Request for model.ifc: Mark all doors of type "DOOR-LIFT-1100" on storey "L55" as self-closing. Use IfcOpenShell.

First a look at what the model holds.

```python
import ifcopenshell
import ifcopenshell.util.element

model = ifcopenshell.open("model.ifc")
print(model.schema)
storey = next(s for s in model.by_type("IfcBuildingStorey") if s.Name == "L55")
doors = [e for e in ifcopenshell.util.element.get_decomposition(storey) if e.is_a("IfcDoor")]
seen = {}
for e in doors:
    element_type = ifcopenshell.util.element.get_type(e)
    key = (element_type.Name if element_type != e and element_type else None, ifcopenshell.util.element.get_pset(e, "Pset_DoorCommon", "SelfClosing"))
    seen[key] = seen.get(key, 0) + 1
for (name, value), count in sorted(seen.items(), key=str):
    print(count, "x", name, "|", value)
```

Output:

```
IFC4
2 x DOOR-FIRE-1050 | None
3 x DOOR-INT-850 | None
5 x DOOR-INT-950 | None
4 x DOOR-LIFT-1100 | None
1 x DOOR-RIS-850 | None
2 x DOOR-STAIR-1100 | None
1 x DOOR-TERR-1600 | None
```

```python
import ifcopenshell
import ifcopenshell.api.pset
import ifcopenshell.util.element

model = ifcopenshell.open("model.ifc")

storey = next(s for s in model.by_type("IfcBuildingStorey") if s.Name == "L55")
doors = [e for e in ifcopenshell.util.element.get_decomposition(storey) if e.is_a("IfcDoor")]

count = 0
for e in doors:
    element_type = ifcopenshell.util.element.get_type(e)
    if element_type in (None, e) or element_type.Name != "DOOR-LIFT-1100":
        continue
    found = ifcopenshell.util.element.get_pset(e, "Pset_DoorCommon", should_inherit=False)
    if found:
        pset = model.by_id(found["id"])
        if len(ifcopenshell.util.element.get_elements_by_pset(pset)) > 1:
            pset = ifcopenshell.api.pset.unshare_pset(model, products=[e], pset=pset)[0]
    else:
        pset = ifcopenshell.api.pset.add_pset(model, product=e, name="Pset_DoorCommon")
    ifcopenshell.api.pset.edit_pset(model, pset=pset, properties={"SelfClosing": True})
    count += 1

print(count, "doors updated")

model.write("model_edited.ifc")
```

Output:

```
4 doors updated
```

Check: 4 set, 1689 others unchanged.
